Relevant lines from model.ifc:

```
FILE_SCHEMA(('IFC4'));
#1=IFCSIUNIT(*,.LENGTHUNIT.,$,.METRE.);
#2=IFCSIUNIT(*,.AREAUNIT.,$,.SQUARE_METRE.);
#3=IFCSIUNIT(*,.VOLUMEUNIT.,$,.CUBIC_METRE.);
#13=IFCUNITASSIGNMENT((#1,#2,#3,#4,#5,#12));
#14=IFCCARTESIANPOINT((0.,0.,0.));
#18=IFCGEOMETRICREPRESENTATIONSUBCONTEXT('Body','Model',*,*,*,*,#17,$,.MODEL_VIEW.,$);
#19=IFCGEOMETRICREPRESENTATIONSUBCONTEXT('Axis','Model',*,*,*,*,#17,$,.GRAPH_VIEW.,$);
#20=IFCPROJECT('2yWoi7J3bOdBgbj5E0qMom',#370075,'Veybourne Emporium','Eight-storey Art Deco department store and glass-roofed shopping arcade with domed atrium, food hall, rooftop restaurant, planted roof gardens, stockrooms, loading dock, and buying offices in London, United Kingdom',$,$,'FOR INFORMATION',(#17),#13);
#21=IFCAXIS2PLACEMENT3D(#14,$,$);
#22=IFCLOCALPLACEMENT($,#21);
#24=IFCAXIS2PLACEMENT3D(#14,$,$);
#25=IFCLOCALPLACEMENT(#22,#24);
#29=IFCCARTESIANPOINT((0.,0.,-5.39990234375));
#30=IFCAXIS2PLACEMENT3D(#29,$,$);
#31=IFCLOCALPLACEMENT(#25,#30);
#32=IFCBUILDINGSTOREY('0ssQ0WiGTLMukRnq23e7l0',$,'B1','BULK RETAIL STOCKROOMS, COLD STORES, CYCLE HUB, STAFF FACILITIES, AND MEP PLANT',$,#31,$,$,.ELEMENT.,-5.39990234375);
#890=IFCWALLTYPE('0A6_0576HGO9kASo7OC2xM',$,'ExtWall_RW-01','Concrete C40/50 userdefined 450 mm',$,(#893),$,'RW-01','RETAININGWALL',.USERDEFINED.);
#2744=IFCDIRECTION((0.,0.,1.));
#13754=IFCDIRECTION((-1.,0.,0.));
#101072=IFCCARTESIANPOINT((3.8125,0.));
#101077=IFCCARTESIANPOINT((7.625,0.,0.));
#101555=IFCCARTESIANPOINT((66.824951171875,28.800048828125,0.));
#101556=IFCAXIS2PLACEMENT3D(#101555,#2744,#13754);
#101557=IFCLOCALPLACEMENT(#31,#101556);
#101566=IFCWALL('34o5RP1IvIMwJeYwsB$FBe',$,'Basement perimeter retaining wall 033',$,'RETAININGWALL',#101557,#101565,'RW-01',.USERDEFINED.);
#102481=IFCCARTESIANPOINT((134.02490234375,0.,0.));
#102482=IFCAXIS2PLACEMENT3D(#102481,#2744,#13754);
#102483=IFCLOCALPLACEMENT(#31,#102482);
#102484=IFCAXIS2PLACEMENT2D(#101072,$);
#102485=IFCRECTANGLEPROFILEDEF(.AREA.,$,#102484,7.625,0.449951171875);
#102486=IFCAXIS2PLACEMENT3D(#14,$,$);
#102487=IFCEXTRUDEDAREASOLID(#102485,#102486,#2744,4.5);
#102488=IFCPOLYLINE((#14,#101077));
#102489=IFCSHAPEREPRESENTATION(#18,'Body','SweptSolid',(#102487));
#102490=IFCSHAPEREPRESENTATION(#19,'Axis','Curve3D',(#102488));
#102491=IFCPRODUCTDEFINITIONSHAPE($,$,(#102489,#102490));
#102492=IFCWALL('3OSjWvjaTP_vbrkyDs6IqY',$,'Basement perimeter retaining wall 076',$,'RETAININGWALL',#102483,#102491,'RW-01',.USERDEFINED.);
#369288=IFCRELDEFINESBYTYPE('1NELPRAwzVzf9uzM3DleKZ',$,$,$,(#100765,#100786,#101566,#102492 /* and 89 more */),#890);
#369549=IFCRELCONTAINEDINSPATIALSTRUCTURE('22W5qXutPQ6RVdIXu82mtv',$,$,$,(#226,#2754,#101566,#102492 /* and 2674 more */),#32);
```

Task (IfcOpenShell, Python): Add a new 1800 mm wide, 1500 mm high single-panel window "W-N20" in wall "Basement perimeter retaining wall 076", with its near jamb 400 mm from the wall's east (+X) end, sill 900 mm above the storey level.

```python
import numpy as np
import ifcopenshell
import ifcopenshell.api.feature
import ifcopenshell.api.geometry
import ifcopenshell.api.root
import ifcopenshell.api.spatial
import ifcopenshell.geom
import ifcopenshell.util.element
import ifcopenshell.util.placement
import ifcopenshell.util.representation
import ifcopenshell.util.shape
import ifcopenshell.util.unit

model = ifcopenshell.open("model.ifc")
unit_scale = ifcopenshell.util.unit.calculate_unit_scale(model)
settings = ifcopenshell.geom.settings()


def volume(element):
    """Net volume in cubic metres, openings subtracted."""
    shape = ifcopenshell.geom.create_shape(settings, element)
    return ifcopenshell.util.shape.get_volume(shape.geometry)


wall = model.by_guid("3OSjWvjaTP_vbrkyDs6IqY")
storey = ifcopenshell.util.element.get_container(wall, ifc_class="IfcBuildingStorey")
context = ifcopenshell.util.representation.get_context(model, "Model", "Body", "MODEL_VIEW")
before = volume(wall)

width, height, from_end, sill = 1.8, 1.5, 0.4, 0.9  # metres

# The wall runs along its own X axis, and the end named is its -X end.
wall_shape = ifcopenshell.geom.create_shape(settings, wall)
x, y, z = ifcopenshell.util.shape.get_vertices(wall_shape.geometry).T
start = x.min() + from_end
face, thickness = float(y.min()), float(y.max() - y.min())
wall_matrix = ifcopenshell.util.placement.get_local_placement(wall.ObjectPlacement)
level = ifcopenshell.util.placement.get_local_placement(storey.ObjectPlacement)[2, 3]


def in_wall(x, y):
    """Placement at x, y metres in the wall's axes, at sill height."""
    matrix = wall_matrix.copy()
    matrix[:, 3] = wall_matrix @ np.array([x / unit_scale, y / unit_scale, 0.0, 1.0])
    matrix[2, 3] = level + sill / unit_scale
    return matrix


# Opening: a box that overshoots both wall faces by 50 mm.
opening = ifcopenshell.api.root.create_entity(model, ifc_class="IfcOpeningElement", predefined_type="OPENING")
box = ifcopenshell.api.geometry.add_wall_representation(
    model, context=context, length=width, height=height, thickness=thickness + 0.1
)
ifcopenshell.api.geometry.assign_representation(model, product=opening, representation=box)
ifcopenshell.api.geometry.edit_object_placement(model, product=opening, matrix=in_wall(start, face - 0.05), is_si=False)
ifcopenshell.api.feature.add_feature(model, feature=opening, element=wall)

window = ifcopenshell.api.root.create_entity(model, ifc_class="IfcWindow", name="W-N20", predefined_type="WINDOW")
window.OverallWidth, window.OverallHeight = width / unit_scale, height / unit_scale
window.PartitioningType = "SINGLE_PANEL"
body = ifcopenshell.api.geometry.add_window_representation(
    model,
    context=context,
    overall_width=window.OverallWidth,
    overall_height=window.OverallHeight,
    partition_type="SINGLE_PANEL",
)
ifcopenshell.api.geometry.assign_representation(model, product=window, representation=body)
ifcopenshell.api.spatial.assign_container(model, products=[window], relating_structure=storey)
ifcopenshell.api.feature.add_filling(model, opening=opening, element=window)

# Centre the window in the wall's thickness.
ifcopenshell.api.geometry.edit_object_placement(model, product=window, matrix=in_wall(start, face), is_si=False)
window_shape = ifcopenshell.geom.create_shape(settings, window)
depth = ifcopenshell.util.shape.get_vertices(window_shape.geometry)[:, 1]
offset = face + thickness / 2 - (depth.min() + depth.max()) / 2
ifcopenshell.api.geometry.edit_object_placement(model, product=window, matrix=in_wall(start, offset), is_si=False)

after = volume(wall)

print(f"wall volume {before:.3f} -> {after:.3f} m3")

model.write("model_edited.ifc")
```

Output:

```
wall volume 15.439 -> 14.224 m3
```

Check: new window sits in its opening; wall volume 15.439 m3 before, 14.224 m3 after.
